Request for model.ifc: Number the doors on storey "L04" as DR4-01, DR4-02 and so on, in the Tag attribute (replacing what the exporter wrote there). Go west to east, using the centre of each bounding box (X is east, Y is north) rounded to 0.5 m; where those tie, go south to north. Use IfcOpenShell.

First a look at what the model holds.

```python
import ifcopenshell
import ifcopenshell.util.element
import ifcopenshell.util.placement

model = ifcopenshell.open("model.ifc")
print(model.schema)
storey = next(s for s in model.by_type("IfcBuildingStorey") if s.Name == "L04")
doors = [e for e in ifcopenshell.util.element.get_decomposition(storey) if e.is_a("IfcDoor")]
for e in sorted(doors, key=lambda e: e.id()):
    origin = ifcopenshell.util.placement.get_local_placement(e.ObjectPlacement)[:3, 3]
    print(e.id(), e.Tag, e.Name, origin.round(2) + 0.0, sep=" | ")
```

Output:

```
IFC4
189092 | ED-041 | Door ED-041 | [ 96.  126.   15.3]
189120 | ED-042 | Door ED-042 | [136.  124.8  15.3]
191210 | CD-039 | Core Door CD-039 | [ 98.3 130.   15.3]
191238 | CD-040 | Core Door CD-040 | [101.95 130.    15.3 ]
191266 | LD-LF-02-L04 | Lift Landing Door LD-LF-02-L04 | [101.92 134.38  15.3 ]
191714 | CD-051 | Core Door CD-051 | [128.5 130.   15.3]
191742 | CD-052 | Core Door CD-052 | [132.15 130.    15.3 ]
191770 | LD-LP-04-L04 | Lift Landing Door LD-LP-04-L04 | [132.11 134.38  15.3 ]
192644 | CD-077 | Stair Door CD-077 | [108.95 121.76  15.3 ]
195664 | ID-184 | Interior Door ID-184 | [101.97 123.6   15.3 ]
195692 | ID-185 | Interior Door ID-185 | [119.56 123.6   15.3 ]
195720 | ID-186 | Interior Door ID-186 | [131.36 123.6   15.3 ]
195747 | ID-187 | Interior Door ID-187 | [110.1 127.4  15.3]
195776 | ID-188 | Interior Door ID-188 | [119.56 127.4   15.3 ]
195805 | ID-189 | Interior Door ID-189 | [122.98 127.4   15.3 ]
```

```python
import ifcopenshell
import ifcopenshell.geom
import ifcopenshell.util.element
import ifcopenshell.util.shape

model = ifcopenshell.open("model.ifc")
settings = ifcopenshell.geom.settings()
settings.set("use-world-coords", True)


def centre(element):
    shape = ifcopenshell.geom.create_shape(settings, element)
    return ifcopenshell.util.shape.get_bbox_centroid(shape.geometry)


storey = next(s for s in model.by_type("IfcBuildingStorey") if s.Name == "L04")
doors = [e for e in ifcopenshell.util.element.get_decomposition(storey) if e.is_a("IfcDoor")]

# Insertion points can sit at a corner or the storey origin, so sort by the geometry (in metres).
centres = {e: centre(e) for e in doors}
doors.sort(key=lambda e: (round(centres[e][0] / 0.5), centres[e][1]))

for i, e in enumerate(doors, start=1):
    number = f"DR4-{i:02d}"
    e.Tag = number
    print(e.id(), number)

model.write("model_v2.ifc")
```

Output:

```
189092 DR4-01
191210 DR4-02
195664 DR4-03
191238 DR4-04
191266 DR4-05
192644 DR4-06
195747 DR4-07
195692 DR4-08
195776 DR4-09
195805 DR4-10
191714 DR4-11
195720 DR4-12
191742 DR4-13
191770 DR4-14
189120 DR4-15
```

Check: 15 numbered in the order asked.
